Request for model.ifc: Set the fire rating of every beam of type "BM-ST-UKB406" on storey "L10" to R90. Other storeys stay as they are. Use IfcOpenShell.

First a look at what the model holds.

```python
import ifcopenshell
import ifcopenshell.util.element

model = ifcopenshell.open("model.ifc")
print(model.schema)
storey = next(s for s in model.by_type("IfcBuildingStorey") if s.Name == "L10")
beams = [e for e in ifcopenshell.util.element.get_decomposition(storey) if e.is_a("IfcBeam")]
seen = {}
for e in beams:
    element_type = ifcopenshell.util.element.get_type(e)
    key = (element_type.Name if element_type != e and element_type else None, ifcopenshell.util.element.get_pset(e, "Pset_BeamCommon", "FireRating"))
    seen[key] = seen.get(key, 0) + 1
for (name, value), count in sorted(seen.items(), key=str):
    print(count, "x", name, "|", value)
```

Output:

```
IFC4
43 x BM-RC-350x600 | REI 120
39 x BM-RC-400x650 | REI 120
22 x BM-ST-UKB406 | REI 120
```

```python
import ifcopenshell
import ifcopenshell.api.pset
import ifcopenshell.util.element

model = ifcopenshell.open("model.ifc")

storey = next(s for s in model.by_type("IfcBuildingStorey") if s.Name == "L10")
beams = [e for e in ifcopenshell.util.element.get_decomposition(storey) if e.is_a("IfcBeam")]

count = 0
for e in beams:
    element_type = ifcopenshell.util.element.get_type(e)
    if element_type in (None, e) or element_type.Name != "BM-ST-UKB406":
        continue
    # add_pset returns the element's existing set when there is one.
    pset = ifcopenshell.api.pset.add_pset(model, product=e, name="Pset_BeamCommon")
    ifcopenshell.api.pset.edit_pset(model, pset=pset, properties={"FireRating": "R90"})
    count += 1

print(count, "beams updated")

model.write("model_edited.ifc")
```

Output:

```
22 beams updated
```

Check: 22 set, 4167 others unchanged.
